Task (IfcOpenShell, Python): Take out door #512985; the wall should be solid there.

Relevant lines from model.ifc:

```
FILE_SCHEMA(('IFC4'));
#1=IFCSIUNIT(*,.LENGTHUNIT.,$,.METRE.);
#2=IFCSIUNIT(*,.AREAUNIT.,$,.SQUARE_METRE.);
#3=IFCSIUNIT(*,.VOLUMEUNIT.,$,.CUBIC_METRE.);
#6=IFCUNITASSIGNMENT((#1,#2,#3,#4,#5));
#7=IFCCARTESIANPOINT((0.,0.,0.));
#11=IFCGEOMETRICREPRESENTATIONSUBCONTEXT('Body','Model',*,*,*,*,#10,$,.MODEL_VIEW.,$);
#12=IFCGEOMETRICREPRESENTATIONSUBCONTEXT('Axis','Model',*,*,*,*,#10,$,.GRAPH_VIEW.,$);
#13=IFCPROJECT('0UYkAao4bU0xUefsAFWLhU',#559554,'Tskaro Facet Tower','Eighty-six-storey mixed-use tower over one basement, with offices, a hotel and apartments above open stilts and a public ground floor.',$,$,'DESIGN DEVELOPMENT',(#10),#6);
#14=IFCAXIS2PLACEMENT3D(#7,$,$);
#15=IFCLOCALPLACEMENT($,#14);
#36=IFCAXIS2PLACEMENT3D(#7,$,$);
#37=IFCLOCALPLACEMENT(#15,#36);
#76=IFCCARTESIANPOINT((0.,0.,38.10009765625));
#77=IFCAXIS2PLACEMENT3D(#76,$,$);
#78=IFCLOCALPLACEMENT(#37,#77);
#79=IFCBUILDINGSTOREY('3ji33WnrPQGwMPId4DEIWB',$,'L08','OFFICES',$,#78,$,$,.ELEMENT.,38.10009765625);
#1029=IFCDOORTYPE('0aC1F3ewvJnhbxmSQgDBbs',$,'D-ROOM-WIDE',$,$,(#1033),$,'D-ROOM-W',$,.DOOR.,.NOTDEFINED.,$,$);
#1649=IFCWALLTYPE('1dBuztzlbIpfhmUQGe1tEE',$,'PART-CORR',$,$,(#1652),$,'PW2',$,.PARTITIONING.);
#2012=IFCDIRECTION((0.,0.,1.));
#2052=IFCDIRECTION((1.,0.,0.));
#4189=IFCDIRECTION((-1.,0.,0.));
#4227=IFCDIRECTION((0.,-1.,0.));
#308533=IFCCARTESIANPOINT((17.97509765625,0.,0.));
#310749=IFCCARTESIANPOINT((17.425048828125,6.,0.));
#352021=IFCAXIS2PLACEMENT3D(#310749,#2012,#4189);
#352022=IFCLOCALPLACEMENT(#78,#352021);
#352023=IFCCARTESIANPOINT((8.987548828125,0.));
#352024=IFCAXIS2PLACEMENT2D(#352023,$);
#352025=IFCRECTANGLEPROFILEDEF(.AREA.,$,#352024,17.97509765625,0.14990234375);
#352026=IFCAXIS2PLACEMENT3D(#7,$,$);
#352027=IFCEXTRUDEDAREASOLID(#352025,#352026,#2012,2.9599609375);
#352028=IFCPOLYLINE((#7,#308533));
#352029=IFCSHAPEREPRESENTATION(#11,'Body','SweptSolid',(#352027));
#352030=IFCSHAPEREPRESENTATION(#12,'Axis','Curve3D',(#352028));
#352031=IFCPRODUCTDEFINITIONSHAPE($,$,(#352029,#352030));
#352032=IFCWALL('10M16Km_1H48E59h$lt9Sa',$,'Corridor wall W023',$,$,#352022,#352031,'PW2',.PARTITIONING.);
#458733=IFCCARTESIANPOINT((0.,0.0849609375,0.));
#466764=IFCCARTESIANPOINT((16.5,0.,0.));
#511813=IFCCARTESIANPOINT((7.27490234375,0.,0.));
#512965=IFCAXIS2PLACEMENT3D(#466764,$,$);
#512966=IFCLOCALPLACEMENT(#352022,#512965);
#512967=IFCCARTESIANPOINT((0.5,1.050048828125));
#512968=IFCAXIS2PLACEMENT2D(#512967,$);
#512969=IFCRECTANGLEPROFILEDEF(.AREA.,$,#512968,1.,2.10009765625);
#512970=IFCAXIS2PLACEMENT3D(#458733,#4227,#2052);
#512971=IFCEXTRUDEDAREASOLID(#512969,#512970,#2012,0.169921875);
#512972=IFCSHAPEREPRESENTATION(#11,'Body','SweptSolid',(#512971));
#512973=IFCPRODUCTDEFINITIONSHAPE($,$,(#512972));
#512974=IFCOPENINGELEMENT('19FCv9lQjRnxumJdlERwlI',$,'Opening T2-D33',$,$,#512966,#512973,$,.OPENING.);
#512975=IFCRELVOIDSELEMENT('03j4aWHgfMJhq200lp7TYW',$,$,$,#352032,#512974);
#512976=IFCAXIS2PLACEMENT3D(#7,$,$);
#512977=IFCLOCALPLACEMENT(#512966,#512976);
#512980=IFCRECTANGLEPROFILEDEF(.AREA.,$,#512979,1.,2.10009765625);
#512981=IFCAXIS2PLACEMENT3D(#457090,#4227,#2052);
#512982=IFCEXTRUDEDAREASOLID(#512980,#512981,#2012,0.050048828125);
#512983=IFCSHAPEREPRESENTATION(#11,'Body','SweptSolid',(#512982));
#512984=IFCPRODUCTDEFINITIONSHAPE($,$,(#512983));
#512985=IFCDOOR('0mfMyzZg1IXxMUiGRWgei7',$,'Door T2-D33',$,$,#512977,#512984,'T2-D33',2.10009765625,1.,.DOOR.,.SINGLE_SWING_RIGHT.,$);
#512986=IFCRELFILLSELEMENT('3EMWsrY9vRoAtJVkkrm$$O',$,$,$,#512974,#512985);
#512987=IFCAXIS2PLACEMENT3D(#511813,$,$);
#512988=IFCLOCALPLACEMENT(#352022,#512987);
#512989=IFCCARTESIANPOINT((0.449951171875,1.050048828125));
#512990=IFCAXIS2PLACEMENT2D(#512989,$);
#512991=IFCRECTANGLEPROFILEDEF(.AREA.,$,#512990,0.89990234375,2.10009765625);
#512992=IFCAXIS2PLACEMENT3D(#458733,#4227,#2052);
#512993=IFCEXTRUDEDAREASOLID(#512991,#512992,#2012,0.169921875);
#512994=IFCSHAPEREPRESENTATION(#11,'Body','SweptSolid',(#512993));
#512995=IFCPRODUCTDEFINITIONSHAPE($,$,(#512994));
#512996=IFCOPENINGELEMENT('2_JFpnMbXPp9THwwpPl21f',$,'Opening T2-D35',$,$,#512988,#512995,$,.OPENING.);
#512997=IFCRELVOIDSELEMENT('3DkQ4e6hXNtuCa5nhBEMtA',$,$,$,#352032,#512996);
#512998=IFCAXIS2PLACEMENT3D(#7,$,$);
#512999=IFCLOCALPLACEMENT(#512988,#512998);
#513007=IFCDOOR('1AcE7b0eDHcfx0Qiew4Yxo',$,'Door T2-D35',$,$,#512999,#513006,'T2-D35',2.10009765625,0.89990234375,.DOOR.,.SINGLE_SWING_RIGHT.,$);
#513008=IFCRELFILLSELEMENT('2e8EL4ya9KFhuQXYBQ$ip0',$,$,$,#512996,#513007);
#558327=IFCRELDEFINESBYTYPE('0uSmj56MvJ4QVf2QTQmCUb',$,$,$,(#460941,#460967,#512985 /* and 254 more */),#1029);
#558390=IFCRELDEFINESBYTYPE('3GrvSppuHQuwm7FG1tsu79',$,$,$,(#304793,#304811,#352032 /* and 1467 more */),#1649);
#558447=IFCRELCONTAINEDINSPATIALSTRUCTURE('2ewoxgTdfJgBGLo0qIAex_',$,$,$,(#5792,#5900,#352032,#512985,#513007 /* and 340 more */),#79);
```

```python
import ifcopenshell
import ifcopenshell.api.feature
import ifcopenshell.api.root
import ifcopenshell.geom
import ifcopenshell.util.shape

model = ifcopenshell.open("model.ifc")
settings = ifcopenshell.geom.settings()


def volume(element):
    """Net volume in cubic metres, openings subtracted."""
    shape = ifcopenshell.geom.create_shape(settings, element)
    return ifcopenshell.util.shape.get_volume(shape.geometry)


door = model.by_guid("0mfMyzZg1IXxMUiGRWgei7")
opening = door.FillsVoids[0].RelatingOpeningElement
wall = opening.VoidsElements[0].RelatingBuildingElement
before = volume(wall)

ifcopenshell.api.root.remove_product(model, product=door)
ifcopenshell.api.feature.remove_feature(model, feature=opening)

after = volume(wall)

print(f"wall volume {before:.3f} -> {after:.3f} m3")

model.write("model_rev.ifc")
```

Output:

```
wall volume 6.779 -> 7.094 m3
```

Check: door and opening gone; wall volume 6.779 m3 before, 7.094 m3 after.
